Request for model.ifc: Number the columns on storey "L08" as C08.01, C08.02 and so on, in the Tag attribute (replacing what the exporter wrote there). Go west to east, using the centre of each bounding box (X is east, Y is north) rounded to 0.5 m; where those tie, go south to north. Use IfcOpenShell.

First a look at what the model holds.

```python
import ifcopenshell
import ifcopenshell.util.element
import ifcopenshell.util.placement

model = ifcopenshell.open("model.ifc")
print(model.schema)
storey = next(s for s in model.by_type("IfcBuildingStorey") if s.Name == "L08")
columns = [e for e in ifcopenshell.util.element.get_decomposition(storey) if e.is_a("IfcColumn")]
for e in sorted(columns, key=lambda e: e.id()):
    origin = ifcopenshell.util.placement.get_local_placement(e.ObjectPlacement)[:3, 3]
    print(e.id(), e.Tag, e.Name, origin.round(2) + 0.0, sep=" | ")
```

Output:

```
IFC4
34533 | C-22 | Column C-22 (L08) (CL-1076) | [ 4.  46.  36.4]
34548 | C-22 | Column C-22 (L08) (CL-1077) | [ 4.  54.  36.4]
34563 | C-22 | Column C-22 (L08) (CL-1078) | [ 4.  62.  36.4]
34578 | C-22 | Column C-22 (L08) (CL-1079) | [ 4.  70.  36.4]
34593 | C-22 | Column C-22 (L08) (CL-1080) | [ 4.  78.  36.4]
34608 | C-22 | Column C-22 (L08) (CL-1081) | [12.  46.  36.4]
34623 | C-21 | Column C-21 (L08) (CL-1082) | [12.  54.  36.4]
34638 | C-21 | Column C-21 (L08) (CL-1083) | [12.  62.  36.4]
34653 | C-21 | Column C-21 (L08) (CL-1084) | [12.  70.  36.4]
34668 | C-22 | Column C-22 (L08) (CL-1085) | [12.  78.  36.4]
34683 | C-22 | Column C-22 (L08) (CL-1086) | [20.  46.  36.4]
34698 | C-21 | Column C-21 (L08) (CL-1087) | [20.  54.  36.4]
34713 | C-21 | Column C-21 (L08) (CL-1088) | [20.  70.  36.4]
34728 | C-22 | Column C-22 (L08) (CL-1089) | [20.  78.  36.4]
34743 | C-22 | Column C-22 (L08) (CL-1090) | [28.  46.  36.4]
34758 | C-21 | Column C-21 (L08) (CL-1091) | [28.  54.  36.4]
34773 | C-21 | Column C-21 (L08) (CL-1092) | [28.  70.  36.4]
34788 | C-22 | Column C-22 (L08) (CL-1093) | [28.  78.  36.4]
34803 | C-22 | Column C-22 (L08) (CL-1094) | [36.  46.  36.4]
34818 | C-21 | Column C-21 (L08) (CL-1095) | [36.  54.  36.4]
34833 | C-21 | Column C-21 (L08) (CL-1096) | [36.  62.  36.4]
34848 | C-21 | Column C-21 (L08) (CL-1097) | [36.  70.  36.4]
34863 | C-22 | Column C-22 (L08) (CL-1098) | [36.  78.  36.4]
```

```python
import ifcopenshell
import ifcopenshell.geom
import ifcopenshell.util.element
import ifcopenshell.util.shape

model = ifcopenshell.open("model.ifc")
settings = ifcopenshell.geom.settings()
settings.set("use-world-coords", True)


def centre(element):
    shape = ifcopenshell.geom.create_shape(settings, element)
    return ifcopenshell.util.shape.get_bbox_centroid(shape.geometry)


storey = next(s for s in model.by_type("IfcBuildingStorey") if s.Name == "L08")
columns = [e for e in ifcopenshell.util.element.get_decomposition(storey) if e.is_a("IfcColumn")]

# Insertion points can sit at a corner or the storey origin, so sort by the geometry (in metres).
centres = {e: centre(e) for e in columns}
columns.sort(key=lambda e: (round(centres[e][0] / 0.5), centres[e][1]))

for i, e in enumerate(columns, start=1):
    number = f"C08.{i:02d}"
    e.Tag = number
    print(e.id(), number)

model.write("model_rev.ifc")
```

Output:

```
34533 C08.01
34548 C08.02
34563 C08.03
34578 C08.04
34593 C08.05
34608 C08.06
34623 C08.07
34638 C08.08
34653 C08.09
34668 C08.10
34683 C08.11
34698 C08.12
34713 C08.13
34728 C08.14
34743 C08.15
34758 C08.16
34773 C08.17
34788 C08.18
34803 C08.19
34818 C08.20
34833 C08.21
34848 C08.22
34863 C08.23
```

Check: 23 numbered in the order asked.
